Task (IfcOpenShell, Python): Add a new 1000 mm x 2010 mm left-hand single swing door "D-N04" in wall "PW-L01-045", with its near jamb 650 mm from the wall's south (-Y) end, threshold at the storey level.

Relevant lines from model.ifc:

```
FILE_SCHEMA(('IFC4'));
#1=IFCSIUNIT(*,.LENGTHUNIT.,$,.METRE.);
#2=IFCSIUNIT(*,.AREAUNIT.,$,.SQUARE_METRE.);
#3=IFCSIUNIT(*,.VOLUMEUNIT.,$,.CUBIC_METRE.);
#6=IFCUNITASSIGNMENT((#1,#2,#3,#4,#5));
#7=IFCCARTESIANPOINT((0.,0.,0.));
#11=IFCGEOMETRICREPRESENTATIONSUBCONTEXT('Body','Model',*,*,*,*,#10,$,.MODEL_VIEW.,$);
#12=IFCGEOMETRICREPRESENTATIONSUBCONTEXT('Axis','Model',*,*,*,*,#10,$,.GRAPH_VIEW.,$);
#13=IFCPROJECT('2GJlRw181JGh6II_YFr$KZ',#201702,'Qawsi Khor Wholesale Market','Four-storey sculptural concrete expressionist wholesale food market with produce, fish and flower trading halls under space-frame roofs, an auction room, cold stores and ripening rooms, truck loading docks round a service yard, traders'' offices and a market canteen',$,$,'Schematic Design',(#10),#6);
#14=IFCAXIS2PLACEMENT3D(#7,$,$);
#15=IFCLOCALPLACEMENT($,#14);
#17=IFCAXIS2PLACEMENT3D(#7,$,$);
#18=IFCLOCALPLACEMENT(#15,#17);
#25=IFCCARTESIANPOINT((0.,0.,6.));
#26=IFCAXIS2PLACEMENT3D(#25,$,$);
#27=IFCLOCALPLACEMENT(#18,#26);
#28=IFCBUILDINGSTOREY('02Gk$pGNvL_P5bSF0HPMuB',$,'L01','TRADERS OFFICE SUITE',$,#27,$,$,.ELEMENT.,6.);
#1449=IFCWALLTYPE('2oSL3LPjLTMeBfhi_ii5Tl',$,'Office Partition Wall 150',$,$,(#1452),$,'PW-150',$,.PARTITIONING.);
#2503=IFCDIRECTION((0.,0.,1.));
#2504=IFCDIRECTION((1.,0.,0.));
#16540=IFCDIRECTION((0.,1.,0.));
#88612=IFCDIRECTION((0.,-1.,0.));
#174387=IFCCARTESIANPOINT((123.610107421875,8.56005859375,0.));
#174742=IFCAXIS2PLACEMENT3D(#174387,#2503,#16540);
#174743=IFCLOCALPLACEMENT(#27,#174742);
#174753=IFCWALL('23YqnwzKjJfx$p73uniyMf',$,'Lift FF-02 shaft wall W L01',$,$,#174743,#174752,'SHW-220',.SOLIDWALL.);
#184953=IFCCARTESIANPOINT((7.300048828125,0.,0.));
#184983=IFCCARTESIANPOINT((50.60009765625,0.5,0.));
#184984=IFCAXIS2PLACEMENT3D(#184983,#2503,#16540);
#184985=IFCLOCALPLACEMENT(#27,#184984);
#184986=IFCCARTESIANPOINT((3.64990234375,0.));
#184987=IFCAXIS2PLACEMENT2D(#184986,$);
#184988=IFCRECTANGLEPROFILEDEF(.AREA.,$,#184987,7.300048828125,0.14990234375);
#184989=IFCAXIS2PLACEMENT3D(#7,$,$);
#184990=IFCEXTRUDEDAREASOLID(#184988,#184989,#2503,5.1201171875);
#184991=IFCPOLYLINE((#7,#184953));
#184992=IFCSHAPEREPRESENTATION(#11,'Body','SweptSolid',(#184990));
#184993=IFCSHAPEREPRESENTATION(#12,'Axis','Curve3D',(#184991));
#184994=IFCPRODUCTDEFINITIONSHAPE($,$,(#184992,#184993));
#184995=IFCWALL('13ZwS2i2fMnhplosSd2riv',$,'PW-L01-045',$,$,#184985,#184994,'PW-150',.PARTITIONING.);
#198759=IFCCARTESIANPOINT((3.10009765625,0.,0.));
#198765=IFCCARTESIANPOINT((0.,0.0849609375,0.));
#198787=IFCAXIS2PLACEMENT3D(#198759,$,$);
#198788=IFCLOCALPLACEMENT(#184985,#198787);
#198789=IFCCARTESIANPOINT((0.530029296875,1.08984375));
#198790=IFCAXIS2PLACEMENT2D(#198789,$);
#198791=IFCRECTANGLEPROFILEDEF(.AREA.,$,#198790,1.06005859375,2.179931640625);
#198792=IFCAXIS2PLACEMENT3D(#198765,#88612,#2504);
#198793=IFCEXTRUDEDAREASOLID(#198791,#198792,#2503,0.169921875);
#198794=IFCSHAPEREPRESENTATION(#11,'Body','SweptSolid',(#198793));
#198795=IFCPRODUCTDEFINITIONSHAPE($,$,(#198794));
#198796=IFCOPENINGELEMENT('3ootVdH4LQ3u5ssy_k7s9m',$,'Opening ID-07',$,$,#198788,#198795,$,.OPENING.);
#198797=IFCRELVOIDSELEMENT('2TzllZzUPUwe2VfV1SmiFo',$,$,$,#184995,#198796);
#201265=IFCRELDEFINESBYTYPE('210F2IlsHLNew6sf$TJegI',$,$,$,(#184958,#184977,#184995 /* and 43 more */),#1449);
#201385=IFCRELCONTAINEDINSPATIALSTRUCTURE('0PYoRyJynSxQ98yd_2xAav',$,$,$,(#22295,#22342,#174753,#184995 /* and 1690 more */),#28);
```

```python
import numpy as np
import ifcopenshell
import ifcopenshell.api.feature
import ifcopenshell.api.geometry
import ifcopenshell.api.root
import ifcopenshell.api.spatial
import ifcopenshell.geom
import ifcopenshell.util.element
import ifcopenshell.util.placement
import ifcopenshell.util.representation
import ifcopenshell.util.shape
import ifcopenshell.util.unit

model = ifcopenshell.open("model.ifc")
unit_scale = ifcopenshell.util.unit.calculate_unit_scale(model)
settings = ifcopenshell.geom.settings()


def volume(element):
    """Net volume in cubic metres, openings subtracted."""
    shape = ifcopenshell.geom.create_shape(settings, element)
    return ifcopenshell.util.shape.get_volume(shape.geometry)


wall = model.by_guid("13ZwS2i2fMnhplosSd2riv")
storey = ifcopenshell.util.element.get_container(wall, ifc_class="IfcBuildingStorey")
context = ifcopenshell.util.representation.get_context(model, "Model", "Body", "MODEL_VIEW")
before = volume(wall)

width, height, from_end, sill = 1, 2.01, 0.65, 0.0  # metres

# The wall runs along its own X axis, and the end named is its -X end.
wall_shape = ifcopenshell.geom.create_shape(settings, wall)
x, y, z = ifcopenshell.util.shape.get_vertices(wall_shape.geometry).T
start = x.min() + from_end
face, thickness = float(y.min()), float(y.max() - y.min())
wall_matrix = ifcopenshell.util.placement.get_local_placement(wall.ObjectPlacement)
level = ifcopenshell.util.placement.get_local_placement(storey.ObjectPlacement)[2, 3]


def in_wall(x, y):
    """Placement at x, y metres in the wall's axes, at sill height."""
    matrix = wall_matrix.copy()
    matrix[:, 3] = wall_matrix @ np.array([x / unit_scale, y / unit_scale, 0.0, 1.0])
    matrix[2, 3] = level + sill / unit_scale
    return matrix


# Opening: a box that overshoots both wall faces by 50 mm.
opening = ifcopenshell.api.root.create_entity(model, ifc_class="IfcOpeningElement", predefined_type="OPENING")
box = ifcopenshell.api.geometry.add_wall_representation(
    model, context=context, length=width, height=height, thickness=thickness + 0.1
)
ifcopenshell.api.geometry.assign_representation(model, product=opening, representation=box)
ifcopenshell.api.geometry.edit_object_placement(model, product=opening, matrix=in_wall(start, face - 0.05), is_si=False)
ifcopenshell.api.feature.add_feature(model, feature=opening, element=wall)

door = ifcopenshell.api.root.create_entity(model, ifc_class="IfcDoor", name="D-N04", predefined_type="DOOR")
door.OverallWidth, door.OverallHeight = width / unit_scale, height / unit_scale
door.OperationType = "SINGLE_SWING_LEFT"
body = ifcopenshell.api.geometry.add_door_representation(
    model,
    context=context,
    overall_width=door.OverallWidth,
    overall_height=door.OverallHeight,
    operation_type="SINGLE_SWING_LEFT",
    lining_properties={"LiningDepth": thickness / unit_scale, "ThresholdDepth": thickness / unit_scale},
)
ifcopenshell.api.geometry.assign_representation(model, product=door, representation=body)
ifcopenshell.api.spatial.assign_container(model, products=[door], relating_structure=storey)
ifcopenshell.api.feature.add_filling(model, opening=opening, element=door)

# The lining spans the wall, so the door starts at the wall face.
ifcopenshell.api.geometry.edit_object_placement(model, product=door, matrix=in_wall(start, face), is_si=False)

after = volume(wall)

print(f"wall volume {before:.3f} -> {after:.3f} m3")

model.write("model_updated.ifc")
```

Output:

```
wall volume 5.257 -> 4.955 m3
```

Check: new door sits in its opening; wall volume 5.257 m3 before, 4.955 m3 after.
